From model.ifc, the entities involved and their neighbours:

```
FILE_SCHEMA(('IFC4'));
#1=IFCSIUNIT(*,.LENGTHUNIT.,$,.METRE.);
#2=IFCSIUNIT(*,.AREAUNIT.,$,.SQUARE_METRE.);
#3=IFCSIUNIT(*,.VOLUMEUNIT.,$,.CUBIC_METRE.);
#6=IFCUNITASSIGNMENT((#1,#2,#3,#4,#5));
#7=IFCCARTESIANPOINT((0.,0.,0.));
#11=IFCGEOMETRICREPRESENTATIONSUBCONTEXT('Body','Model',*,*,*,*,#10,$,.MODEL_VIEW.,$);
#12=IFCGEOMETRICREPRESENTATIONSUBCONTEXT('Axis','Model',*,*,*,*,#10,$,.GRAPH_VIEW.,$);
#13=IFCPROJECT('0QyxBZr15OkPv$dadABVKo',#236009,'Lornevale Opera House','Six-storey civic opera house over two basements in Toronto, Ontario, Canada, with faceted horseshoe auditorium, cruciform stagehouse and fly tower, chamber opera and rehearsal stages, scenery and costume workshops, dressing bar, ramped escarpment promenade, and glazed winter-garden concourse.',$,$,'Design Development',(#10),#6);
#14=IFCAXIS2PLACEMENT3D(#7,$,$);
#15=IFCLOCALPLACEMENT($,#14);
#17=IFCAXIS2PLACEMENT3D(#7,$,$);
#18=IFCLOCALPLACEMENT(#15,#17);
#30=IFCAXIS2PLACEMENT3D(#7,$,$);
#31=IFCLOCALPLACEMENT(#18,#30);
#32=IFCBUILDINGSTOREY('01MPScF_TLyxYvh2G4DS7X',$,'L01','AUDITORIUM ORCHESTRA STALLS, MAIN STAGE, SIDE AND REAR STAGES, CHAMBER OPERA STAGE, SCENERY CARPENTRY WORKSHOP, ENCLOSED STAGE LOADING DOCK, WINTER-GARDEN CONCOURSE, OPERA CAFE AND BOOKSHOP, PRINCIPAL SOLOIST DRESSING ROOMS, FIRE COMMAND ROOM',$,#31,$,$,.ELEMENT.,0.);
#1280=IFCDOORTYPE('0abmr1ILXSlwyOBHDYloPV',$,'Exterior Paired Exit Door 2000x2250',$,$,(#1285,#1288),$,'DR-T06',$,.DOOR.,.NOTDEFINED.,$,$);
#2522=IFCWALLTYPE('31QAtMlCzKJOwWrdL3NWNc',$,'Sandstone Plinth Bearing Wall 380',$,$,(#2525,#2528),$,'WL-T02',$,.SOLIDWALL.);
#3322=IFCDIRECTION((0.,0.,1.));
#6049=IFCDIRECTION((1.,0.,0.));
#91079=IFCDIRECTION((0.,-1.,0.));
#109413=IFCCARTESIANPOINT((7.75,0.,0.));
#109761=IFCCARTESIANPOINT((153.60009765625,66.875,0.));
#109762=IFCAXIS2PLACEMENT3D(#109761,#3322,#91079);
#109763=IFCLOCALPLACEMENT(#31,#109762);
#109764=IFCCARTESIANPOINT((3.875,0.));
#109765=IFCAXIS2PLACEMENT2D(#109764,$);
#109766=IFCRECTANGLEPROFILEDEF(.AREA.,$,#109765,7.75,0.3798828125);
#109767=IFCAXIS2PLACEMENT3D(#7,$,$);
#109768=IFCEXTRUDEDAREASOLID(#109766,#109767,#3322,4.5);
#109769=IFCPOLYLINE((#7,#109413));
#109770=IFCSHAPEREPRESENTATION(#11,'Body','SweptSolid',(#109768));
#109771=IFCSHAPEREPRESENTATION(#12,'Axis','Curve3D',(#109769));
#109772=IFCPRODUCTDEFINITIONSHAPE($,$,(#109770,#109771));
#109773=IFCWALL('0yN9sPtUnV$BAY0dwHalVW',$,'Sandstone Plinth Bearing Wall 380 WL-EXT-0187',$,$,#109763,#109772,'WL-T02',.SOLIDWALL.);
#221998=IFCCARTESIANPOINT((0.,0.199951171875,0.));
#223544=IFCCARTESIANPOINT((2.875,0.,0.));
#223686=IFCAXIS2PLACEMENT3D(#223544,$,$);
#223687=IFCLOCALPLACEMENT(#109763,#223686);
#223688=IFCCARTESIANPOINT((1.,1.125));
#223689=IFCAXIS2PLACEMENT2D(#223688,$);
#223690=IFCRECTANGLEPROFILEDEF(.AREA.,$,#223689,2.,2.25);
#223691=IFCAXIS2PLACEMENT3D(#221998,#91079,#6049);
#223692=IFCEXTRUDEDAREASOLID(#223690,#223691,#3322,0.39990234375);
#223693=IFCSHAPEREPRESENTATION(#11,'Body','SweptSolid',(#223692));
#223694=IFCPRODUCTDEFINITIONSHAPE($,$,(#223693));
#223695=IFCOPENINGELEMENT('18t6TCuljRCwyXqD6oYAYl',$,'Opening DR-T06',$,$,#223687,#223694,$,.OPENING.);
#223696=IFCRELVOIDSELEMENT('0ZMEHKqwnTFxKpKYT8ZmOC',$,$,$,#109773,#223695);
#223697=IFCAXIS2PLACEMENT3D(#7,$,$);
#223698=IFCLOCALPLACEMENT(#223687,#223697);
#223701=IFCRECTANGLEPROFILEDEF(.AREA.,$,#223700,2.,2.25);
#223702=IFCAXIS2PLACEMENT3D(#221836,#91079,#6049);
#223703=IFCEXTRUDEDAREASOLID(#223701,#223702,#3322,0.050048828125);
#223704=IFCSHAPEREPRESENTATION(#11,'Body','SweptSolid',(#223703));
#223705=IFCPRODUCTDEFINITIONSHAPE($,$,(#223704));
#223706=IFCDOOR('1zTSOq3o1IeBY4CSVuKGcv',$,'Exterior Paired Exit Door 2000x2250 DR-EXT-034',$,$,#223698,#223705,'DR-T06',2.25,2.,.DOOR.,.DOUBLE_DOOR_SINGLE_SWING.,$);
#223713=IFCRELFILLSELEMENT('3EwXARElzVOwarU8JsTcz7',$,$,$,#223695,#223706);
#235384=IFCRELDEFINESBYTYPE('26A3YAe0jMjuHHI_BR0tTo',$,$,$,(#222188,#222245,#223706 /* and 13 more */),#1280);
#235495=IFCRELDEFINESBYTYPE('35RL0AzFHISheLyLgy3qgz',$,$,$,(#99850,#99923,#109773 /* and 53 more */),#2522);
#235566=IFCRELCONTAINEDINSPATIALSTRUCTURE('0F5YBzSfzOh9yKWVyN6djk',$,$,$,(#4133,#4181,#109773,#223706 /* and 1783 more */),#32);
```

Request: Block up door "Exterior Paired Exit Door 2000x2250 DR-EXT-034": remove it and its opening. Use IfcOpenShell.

```python
import ifcopenshell
import ifcopenshell.api.feature
import ifcopenshell.api.root
import ifcopenshell.geom
import ifcopenshell.util.shape

model = ifcopenshell.open("model.ifc")
settings = ifcopenshell.geom.settings()


def volume(element):
    """Net volume in cubic metres, openings subtracted."""
    shape = ifcopenshell.geom.create_shape(settings, element)
    return ifcopenshell.util.shape.get_volume(shape.geometry)


door = model.by_guid("1zTSOq3o1IeBY4CSVuKGcv")
opening = door.FillsVoids[0].RelatingOpeningElement
wall = opening.VoidsElements[0].RelatingBuildingElement
before = volume(wall)

ifcopenshell.api.root.remove_product(model, product=door)
ifcopenshell.api.feature.remove_feature(model, feature=opening)

after = volume(wall)

print(f"wall volume {before:.3f} -> {after:.3f} m3")

model.write("model_updated.ifc")
```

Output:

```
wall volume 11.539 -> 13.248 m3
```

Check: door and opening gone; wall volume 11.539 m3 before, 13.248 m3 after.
